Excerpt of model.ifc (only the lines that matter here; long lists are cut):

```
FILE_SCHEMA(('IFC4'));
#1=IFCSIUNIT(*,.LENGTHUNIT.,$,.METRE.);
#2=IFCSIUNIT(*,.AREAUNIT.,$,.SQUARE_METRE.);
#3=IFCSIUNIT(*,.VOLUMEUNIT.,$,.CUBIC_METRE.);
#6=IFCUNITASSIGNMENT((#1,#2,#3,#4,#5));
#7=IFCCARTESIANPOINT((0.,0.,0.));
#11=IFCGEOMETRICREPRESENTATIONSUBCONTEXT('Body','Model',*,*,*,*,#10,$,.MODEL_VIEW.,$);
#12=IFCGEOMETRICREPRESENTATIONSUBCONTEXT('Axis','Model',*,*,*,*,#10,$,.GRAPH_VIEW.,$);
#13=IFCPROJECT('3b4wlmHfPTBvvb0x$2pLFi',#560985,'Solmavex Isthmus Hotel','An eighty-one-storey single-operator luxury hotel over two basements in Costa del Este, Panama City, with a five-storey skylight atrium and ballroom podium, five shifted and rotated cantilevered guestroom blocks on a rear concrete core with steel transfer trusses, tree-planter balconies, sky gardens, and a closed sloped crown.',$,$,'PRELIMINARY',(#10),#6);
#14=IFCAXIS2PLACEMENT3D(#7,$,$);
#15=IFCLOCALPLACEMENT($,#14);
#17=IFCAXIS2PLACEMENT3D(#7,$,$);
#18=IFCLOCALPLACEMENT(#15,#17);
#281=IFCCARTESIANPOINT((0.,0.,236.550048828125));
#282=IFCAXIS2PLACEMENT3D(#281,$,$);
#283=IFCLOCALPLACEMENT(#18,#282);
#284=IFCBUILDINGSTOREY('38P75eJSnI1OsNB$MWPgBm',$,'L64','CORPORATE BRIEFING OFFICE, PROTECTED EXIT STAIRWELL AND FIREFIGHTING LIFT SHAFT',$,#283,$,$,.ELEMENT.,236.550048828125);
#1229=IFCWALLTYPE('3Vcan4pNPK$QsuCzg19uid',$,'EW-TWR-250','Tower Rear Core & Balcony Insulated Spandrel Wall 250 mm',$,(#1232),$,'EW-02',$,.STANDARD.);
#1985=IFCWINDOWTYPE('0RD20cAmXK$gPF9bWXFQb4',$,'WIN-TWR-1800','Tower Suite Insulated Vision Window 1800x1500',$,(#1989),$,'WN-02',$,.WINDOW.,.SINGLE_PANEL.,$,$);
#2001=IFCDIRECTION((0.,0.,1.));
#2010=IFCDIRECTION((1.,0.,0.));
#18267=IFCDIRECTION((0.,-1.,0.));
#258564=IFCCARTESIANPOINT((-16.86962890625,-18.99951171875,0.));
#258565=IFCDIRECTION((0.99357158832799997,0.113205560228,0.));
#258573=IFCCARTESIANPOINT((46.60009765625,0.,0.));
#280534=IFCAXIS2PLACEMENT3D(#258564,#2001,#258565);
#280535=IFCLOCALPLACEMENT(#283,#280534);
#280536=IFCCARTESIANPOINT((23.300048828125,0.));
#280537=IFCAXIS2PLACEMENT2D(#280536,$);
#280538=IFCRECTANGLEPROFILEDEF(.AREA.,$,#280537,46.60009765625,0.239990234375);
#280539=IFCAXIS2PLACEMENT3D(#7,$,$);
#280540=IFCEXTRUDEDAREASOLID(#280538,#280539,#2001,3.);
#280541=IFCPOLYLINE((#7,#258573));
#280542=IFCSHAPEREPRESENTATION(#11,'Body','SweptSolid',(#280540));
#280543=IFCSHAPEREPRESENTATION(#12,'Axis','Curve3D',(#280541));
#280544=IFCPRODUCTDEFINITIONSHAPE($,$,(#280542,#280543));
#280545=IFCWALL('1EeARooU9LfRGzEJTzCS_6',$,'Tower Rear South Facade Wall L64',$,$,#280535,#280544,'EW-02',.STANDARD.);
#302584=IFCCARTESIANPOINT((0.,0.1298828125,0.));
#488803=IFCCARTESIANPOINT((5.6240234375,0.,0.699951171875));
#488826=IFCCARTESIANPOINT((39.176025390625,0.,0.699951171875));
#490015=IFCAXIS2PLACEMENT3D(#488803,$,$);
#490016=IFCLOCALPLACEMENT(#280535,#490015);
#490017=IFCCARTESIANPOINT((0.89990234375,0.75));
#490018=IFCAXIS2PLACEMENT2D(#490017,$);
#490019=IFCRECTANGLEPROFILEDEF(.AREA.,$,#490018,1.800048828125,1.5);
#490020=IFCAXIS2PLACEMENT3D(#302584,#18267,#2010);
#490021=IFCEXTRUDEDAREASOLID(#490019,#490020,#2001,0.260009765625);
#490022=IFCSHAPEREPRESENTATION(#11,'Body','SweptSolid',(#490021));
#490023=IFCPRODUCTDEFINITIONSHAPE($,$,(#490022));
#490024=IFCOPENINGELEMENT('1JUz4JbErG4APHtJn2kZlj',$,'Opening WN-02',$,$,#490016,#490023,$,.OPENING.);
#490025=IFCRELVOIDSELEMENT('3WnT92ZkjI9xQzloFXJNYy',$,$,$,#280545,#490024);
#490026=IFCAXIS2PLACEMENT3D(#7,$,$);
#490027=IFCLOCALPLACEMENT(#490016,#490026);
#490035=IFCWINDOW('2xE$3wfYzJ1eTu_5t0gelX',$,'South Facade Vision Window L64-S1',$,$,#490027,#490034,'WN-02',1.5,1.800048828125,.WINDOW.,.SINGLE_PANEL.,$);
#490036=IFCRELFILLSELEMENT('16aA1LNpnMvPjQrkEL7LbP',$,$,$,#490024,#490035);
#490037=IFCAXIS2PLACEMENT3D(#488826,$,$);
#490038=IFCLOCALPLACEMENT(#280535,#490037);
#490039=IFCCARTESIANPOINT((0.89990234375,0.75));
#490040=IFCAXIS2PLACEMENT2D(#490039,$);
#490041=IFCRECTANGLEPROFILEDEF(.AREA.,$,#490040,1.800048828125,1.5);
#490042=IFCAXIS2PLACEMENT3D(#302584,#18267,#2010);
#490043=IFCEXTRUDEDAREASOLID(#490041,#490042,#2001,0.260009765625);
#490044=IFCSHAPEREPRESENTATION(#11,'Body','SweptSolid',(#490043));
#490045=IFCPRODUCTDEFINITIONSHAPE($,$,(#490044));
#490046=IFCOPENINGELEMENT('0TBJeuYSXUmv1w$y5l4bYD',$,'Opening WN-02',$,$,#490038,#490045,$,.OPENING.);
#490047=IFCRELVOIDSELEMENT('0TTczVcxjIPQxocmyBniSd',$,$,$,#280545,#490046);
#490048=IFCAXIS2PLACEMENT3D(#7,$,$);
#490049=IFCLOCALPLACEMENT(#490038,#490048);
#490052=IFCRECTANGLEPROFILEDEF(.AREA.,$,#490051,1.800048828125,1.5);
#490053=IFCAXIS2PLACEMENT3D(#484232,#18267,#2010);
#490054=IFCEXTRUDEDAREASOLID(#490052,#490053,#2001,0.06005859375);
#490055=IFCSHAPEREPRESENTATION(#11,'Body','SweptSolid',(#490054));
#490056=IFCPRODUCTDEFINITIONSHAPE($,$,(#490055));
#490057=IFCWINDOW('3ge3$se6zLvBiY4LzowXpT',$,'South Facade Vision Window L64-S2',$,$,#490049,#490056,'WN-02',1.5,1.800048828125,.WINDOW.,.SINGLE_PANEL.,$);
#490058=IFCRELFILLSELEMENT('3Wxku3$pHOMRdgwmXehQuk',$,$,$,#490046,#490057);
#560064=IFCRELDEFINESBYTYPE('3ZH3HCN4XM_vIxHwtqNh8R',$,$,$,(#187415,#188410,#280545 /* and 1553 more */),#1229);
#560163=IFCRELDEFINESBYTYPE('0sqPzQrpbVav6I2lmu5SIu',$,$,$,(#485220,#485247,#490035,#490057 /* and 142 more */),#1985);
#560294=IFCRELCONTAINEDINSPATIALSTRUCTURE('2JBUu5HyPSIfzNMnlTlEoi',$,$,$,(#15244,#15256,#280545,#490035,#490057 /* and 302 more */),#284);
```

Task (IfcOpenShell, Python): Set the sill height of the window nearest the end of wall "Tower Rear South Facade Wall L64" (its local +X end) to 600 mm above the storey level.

```python
import numpy as np
import ifcopenshell
import ifcopenshell.api.geometry
import ifcopenshell.geom
import ifcopenshell.util.element
import ifcopenshell.util.placement
import ifcopenshell.util.shape
import ifcopenshell.util.unit

model = ifcopenshell.open("model.ifc")
unit_scale = ifcopenshell.util.unit.calculate_unit_scale(model)

window = model.by_guid("3ge3$se6zLvBiY4LzowXpT")
opening = window.FillsVoids[0].RelatingOpeningElement
storey = ifcopenshell.util.element.get_container(window, ifc_class="IfcBuildingStorey")
level = ifcopenshell.util.placement.get_local_placement(storey.ObjectPlacement)[2, 3]

# The opening's origin need not be at the sill, so measure its lowest point.
shape = ifcopenshell.geom.create_shape(ifcopenshell.geom.settings(), opening)
bottom = ifcopenshell.util.shape.get_shape_bottom_elevation(shape, shape.geometry) / unit_scale
dz = level + 0.6 - bottom

shift = np.array([0.0, 0.0, dz])
# The window is placed relative to its opening, so it follows when the opening moves.
matrix = ifcopenshell.util.placement.get_local_placement(opening.ObjectPlacement)
matrix[:3, 3] += shift
ifcopenshell.api.geometry.edit_object_placement(
    model, product=opening, matrix=matrix, is_si=False, should_transform_children=True
)

print(f"moved by {dz * unit_scale:+.3f} m")

model.write("model_rev.ifc")
```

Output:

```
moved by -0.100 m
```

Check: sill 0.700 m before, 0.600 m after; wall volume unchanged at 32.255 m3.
